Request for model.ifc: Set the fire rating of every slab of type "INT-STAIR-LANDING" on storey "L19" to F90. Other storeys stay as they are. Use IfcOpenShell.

First a look at what the model holds.

```python
import ifcopenshell
import ifcopenshell.util.element

model = ifcopenshell.open("model.ifc")
print(model.schema)
storey = next(s for s in model.by_type("IfcBuildingStorey") if s.Name == "L19")
slabs = [e for e in ifcopenshell.util.element.get_decomposition(storey) if e.is_a("IfcSlab")]
seen = {}
for e in slabs:
    element_type = ifcopenshell.util.element.get_type(e)
    key = (element_type.Name if element_type != e and element_type else None, ifcopenshell.util.element.get_pset(e, "Pset_SlabCommon", "FireRating"))
    seen[key] = seen.get(key, 0) + 1
for (name, value), count in sorted(seen.items(), key=str):
    print(count, "x", name, "|", value)
```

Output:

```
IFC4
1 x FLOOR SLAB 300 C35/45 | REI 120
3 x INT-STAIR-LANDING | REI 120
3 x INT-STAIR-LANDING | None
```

```python
import ifcopenshell
import ifcopenshell.api.pset
import ifcopenshell.util.element

model = ifcopenshell.open("model.ifc")

storey = next(s for s in model.by_type("IfcBuildingStorey") if s.Name == "L19")
slabs = [e for e in ifcopenshell.util.element.get_decomposition(storey) if e.is_a("IfcSlab")]

count = 0
for e in slabs:
    element_type = ifcopenshell.util.element.get_type(e)
    if element_type in (None, e) or element_type.Name != "INT-STAIR-LANDING":
        continue
    found = ifcopenshell.util.element.get_pset(e, "Pset_SlabCommon", should_inherit=False)
    if found:
        pset = model.by_id(found["id"])
        if len(ifcopenshell.util.element.get_elements_by_pset(pset)) > 1:
            pset = ifcopenshell.api.pset.unshare_pset(model, products=[e], pset=pset)[0]
    else:
        pset = ifcopenshell.api.pset.add_pset(model, product=e, name="Pset_SlabCommon")
    ifcopenshell.api.pset.edit_pset(model, pset=pset, properties={"FireRating": "F90"})
    count += 1

print(count, "slabs updated")

model.write("model_updated.ifc")
```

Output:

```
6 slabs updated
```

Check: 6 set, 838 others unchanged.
